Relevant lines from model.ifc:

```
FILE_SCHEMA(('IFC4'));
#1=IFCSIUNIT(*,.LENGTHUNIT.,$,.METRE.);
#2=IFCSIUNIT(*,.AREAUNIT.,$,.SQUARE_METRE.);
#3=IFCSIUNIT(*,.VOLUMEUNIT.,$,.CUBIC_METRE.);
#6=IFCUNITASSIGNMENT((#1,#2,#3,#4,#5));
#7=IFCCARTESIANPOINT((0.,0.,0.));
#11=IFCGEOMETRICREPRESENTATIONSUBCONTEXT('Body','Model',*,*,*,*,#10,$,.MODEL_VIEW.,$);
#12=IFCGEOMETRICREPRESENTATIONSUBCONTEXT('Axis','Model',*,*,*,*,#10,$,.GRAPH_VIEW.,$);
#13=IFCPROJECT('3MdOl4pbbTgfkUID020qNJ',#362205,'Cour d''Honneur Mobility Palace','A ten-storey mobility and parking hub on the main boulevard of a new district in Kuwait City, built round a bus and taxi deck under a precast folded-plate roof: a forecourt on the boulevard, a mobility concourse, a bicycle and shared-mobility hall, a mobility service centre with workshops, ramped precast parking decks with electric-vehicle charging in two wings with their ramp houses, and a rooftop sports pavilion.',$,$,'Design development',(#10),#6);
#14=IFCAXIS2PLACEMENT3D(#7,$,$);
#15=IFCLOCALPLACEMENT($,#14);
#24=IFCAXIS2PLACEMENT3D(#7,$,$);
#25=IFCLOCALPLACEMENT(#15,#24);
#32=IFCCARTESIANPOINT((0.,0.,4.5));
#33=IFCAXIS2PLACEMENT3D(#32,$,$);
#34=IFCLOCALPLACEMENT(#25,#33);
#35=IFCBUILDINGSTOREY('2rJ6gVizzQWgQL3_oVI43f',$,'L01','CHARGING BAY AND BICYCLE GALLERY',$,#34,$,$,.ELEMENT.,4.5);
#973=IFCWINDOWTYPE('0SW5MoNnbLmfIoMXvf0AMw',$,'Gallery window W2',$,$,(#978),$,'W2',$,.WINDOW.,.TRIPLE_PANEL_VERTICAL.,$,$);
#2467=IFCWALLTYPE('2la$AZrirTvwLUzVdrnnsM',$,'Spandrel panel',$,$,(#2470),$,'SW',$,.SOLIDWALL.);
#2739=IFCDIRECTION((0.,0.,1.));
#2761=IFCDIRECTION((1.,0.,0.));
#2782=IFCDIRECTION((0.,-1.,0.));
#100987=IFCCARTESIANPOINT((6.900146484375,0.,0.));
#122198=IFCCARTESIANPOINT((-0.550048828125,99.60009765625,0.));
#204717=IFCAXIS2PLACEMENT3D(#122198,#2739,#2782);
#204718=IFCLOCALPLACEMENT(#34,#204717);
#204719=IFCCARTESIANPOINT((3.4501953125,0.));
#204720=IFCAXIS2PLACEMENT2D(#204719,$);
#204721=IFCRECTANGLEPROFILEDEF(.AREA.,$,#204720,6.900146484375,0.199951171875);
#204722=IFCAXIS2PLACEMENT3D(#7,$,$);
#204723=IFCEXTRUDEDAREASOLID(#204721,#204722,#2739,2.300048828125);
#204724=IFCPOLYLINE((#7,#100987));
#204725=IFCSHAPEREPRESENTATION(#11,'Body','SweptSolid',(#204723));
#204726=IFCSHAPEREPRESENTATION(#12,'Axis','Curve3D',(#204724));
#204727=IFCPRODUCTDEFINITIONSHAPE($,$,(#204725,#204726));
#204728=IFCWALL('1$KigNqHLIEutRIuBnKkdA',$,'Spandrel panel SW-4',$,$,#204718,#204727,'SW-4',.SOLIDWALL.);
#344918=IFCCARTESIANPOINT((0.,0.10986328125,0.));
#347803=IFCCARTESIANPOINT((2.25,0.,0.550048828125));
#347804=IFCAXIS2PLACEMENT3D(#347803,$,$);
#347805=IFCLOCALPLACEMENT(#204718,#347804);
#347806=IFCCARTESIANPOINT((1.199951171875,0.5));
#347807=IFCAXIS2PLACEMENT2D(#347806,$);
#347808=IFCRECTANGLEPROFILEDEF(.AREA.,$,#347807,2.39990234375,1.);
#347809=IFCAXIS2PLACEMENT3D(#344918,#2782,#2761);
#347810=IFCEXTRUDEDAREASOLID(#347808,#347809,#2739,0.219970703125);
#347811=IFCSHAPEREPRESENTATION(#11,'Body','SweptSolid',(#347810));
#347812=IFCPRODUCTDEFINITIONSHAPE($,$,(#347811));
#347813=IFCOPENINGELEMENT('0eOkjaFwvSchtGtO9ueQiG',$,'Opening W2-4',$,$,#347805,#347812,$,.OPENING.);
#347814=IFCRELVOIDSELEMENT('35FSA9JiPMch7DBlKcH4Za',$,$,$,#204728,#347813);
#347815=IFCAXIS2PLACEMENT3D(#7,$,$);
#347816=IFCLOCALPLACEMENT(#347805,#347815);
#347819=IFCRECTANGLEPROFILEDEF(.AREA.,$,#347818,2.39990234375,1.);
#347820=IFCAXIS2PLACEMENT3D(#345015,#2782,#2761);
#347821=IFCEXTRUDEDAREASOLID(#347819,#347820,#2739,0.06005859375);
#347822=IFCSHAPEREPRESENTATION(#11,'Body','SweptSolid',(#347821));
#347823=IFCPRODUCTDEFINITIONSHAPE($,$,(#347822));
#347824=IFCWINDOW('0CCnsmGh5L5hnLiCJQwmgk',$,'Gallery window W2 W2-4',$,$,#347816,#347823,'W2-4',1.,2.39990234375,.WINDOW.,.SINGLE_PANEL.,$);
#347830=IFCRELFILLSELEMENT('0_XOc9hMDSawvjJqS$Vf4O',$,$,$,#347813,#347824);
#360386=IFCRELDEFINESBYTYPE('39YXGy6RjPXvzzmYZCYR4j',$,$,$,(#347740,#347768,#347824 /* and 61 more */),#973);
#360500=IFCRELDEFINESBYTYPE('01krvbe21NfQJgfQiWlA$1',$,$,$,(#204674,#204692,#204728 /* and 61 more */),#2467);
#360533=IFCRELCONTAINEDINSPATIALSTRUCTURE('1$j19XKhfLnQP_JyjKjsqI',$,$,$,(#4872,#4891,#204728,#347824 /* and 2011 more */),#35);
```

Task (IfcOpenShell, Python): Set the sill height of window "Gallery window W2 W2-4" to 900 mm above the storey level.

```python
import numpy as np
import ifcopenshell
import ifcopenshell.api.geometry
import ifcopenshell.geom
import ifcopenshell.util.element
import ifcopenshell.util.placement
import ifcopenshell.util.shape
import ifcopenshell.util.unit

model = ifcopenshell.open("model.ifc")
unit_scale = ifcopenshell.util.unit.calculate_unit_scale(model)

window = model.by_guid("0CCnsmGh5L5hnLiCJQwmgk")
opening = window.FillsVoids[0].RelatingOpeningElement
storey = ifcopenshell.util.element.get_container(window, ifc_class="IfcBuildingStorey")
level = ifcopenshell.util.placement.get_local_placement(storey.ObjectPlacement)[2, 3]

# The opening's origin need not be at the sill, so measure its lowest point.
shape = ifcopenshell.geom.create_shape(ifcopenshell.geom.settings(), opening)
bottom = ifcopenshell.util.shape.get_shape_bottom_elevation(shape, shape.geometry) / unit_scale
dz = level + 0.9 / unit_scale - bottom

shift = np.array([0.0, 0.0, dz])
# The window is placed relative to its opening, so it follows when the opening moves.
matrix = ifcopenshell.util.placement.get_local_placement(opening.ObjectPlacement)
matrix[:3, 3] += shift
ifcopenshell.api.geometry.edit_object_placement(
    model, product=opening, matrix=matrix, is_si=False, should_transform_children=True
)

print(f"moved by {dz * unit_scale:+.3f} m")

model.write("model_updated.ifc")
```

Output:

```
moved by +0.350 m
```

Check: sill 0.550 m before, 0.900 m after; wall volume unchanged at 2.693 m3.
